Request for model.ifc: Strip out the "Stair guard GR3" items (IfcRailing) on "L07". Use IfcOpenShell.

First a look at what the model holds.

```python
import ifcopenshell
import ifcopenshell.util.element

model = ifcopenshell.open("model.ifc")
print(model.schema)
storey = next(s for s in model.by_type("IfcBuildingStorey") if s.Name == "L07")
railings = [e for e in ifcopenshell.util.element.get_decomposition(storey) if e.is_a("IfcRailing")]
seen = {}
for e in railings:
    element_type = ifcopenshell.util.element.get_type(e)
    name = element_type.Name if element_type not in (None, e) else None
    seen[name] = seen.get(name, 0) + 1
for name, count in sorted(seen.items(), key=str):
    print(count, "x", name)
```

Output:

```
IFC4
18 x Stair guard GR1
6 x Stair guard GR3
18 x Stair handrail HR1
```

```python
import ifcopenshell
import ifcopenshell.api.root
import ifcopenshell.util.element

model = ifcopenshell.open("model.ifc")

storey = next(s for s in model.by_type("IfcBuildingStorey") if s.Name == "L07")
railings = [e for e in ifcopenshell.util.element.get_decomposition(storey) if e.is_a("IfcRailing")]
targets = [e for e in railings if (t := ifcopenshell.util.element.get_type(e)) not in (None, e) and t.Name == "Stair guard GR3"]

for e in targets:
    ifcopenshell.api.root.remove_product(model, product=e)
print(len(targets), "removed")

model.write("model_updated.ifc")
```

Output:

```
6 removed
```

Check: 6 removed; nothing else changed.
